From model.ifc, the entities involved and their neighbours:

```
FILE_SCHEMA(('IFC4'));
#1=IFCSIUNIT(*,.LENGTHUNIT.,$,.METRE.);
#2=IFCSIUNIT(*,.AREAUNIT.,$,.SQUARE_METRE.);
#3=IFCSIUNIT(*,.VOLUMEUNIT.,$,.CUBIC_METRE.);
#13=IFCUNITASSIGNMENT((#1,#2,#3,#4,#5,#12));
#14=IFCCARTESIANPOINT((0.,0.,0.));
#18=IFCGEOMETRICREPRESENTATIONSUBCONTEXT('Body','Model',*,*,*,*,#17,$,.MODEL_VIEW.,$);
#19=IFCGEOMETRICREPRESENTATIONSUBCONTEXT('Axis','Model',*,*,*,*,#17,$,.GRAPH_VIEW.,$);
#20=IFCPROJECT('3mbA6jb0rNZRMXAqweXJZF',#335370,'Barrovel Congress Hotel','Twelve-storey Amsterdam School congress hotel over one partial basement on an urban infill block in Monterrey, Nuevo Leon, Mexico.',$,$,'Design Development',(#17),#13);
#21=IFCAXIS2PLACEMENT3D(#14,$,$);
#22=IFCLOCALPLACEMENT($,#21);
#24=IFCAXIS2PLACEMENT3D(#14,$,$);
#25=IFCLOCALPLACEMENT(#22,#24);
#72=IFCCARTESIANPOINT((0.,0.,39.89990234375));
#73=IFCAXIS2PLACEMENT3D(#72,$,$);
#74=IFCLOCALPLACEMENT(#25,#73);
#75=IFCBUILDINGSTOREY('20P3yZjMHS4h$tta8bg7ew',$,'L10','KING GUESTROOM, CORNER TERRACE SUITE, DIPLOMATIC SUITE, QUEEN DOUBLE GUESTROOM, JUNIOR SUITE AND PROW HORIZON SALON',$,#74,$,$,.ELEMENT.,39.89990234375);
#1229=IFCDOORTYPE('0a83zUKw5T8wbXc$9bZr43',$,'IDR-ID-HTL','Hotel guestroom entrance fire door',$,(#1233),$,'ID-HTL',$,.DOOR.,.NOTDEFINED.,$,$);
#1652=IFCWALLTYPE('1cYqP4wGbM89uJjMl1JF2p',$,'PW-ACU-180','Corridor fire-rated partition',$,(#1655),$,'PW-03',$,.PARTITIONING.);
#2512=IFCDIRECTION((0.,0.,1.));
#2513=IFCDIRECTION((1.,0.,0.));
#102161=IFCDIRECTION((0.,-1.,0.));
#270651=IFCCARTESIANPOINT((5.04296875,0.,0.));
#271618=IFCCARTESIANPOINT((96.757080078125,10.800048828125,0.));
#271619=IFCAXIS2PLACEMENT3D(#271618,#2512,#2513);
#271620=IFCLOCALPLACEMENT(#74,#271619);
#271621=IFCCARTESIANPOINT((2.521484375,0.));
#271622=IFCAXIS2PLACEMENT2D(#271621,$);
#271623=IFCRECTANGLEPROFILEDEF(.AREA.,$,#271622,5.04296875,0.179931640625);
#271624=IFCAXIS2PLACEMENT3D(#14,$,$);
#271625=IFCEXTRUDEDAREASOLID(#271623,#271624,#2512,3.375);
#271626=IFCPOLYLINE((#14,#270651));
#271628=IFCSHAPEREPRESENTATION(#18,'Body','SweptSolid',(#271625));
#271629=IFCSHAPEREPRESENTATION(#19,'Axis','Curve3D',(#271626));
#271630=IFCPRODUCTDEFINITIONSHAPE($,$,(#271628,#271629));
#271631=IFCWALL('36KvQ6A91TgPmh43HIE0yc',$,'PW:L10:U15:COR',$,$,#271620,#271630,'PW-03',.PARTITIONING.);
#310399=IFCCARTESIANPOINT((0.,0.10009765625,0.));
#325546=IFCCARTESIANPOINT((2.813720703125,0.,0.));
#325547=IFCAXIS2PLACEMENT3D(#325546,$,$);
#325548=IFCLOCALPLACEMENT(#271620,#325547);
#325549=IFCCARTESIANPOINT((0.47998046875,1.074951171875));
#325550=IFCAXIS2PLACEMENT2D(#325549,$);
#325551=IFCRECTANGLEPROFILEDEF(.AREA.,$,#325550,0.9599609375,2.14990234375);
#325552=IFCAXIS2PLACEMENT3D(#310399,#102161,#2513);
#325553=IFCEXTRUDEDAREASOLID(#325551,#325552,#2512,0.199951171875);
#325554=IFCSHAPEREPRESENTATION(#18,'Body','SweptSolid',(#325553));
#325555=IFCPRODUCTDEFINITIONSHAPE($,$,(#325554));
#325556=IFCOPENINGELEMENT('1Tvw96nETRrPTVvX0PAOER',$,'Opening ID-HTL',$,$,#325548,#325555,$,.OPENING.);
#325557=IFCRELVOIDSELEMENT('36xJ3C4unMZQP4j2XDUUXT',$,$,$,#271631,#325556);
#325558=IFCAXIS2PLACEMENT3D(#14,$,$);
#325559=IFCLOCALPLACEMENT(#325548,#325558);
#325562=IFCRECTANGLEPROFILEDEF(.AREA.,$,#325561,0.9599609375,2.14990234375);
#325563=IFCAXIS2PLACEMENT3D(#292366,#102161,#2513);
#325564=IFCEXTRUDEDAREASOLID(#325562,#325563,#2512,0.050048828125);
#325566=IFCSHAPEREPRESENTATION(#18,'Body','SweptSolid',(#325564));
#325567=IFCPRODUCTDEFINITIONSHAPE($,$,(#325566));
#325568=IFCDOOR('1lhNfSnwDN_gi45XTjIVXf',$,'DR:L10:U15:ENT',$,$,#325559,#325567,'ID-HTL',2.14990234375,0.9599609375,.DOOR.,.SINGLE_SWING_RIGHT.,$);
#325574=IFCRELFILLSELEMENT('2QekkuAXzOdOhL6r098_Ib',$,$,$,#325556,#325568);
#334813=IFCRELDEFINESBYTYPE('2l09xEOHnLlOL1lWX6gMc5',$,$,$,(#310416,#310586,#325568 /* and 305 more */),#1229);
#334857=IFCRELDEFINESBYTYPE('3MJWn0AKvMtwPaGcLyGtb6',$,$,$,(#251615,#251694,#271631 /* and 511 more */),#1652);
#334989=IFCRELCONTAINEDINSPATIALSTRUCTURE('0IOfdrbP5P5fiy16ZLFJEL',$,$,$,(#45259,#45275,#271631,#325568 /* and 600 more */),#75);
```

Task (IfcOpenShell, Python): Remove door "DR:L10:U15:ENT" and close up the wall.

```python
import ifcopenshell
import ifcopenshell.api.feature
import ifcopenshell.api.root
import ifcopenshell.geom
import ifcopenshell.util.shape

model = ifcopenshell.open("model.ifc")
settings = ifcopenshell.geom.settings()


def volume(element):
    """Net volume in cubic metres, openings subtracted."""
    shape = ifcopenshell.geom.create_shape(settings, element)
    return ifcopenshell.util.shape.get_volume(shape.geometry)


door = model.by_guid("1lhNfSnwDN_gi45XTjIVXf")
opening = door.FillsVoids[0].RelatingOpeningElement
wall = opening.VoidsElements[0].RelatingBuildingElement
before = volume(wall)

ifcopenshell.api.root.remove_product(model, product=door)
ifcopenshell.api.feature.remove_feature(model, feature=opening)

after = volume(wall)

print(f"wall volume {before:.3f} -> {after:.3f} m3")

model.write("model_updated.ifc")
```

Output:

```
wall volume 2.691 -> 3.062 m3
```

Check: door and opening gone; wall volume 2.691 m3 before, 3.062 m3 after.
